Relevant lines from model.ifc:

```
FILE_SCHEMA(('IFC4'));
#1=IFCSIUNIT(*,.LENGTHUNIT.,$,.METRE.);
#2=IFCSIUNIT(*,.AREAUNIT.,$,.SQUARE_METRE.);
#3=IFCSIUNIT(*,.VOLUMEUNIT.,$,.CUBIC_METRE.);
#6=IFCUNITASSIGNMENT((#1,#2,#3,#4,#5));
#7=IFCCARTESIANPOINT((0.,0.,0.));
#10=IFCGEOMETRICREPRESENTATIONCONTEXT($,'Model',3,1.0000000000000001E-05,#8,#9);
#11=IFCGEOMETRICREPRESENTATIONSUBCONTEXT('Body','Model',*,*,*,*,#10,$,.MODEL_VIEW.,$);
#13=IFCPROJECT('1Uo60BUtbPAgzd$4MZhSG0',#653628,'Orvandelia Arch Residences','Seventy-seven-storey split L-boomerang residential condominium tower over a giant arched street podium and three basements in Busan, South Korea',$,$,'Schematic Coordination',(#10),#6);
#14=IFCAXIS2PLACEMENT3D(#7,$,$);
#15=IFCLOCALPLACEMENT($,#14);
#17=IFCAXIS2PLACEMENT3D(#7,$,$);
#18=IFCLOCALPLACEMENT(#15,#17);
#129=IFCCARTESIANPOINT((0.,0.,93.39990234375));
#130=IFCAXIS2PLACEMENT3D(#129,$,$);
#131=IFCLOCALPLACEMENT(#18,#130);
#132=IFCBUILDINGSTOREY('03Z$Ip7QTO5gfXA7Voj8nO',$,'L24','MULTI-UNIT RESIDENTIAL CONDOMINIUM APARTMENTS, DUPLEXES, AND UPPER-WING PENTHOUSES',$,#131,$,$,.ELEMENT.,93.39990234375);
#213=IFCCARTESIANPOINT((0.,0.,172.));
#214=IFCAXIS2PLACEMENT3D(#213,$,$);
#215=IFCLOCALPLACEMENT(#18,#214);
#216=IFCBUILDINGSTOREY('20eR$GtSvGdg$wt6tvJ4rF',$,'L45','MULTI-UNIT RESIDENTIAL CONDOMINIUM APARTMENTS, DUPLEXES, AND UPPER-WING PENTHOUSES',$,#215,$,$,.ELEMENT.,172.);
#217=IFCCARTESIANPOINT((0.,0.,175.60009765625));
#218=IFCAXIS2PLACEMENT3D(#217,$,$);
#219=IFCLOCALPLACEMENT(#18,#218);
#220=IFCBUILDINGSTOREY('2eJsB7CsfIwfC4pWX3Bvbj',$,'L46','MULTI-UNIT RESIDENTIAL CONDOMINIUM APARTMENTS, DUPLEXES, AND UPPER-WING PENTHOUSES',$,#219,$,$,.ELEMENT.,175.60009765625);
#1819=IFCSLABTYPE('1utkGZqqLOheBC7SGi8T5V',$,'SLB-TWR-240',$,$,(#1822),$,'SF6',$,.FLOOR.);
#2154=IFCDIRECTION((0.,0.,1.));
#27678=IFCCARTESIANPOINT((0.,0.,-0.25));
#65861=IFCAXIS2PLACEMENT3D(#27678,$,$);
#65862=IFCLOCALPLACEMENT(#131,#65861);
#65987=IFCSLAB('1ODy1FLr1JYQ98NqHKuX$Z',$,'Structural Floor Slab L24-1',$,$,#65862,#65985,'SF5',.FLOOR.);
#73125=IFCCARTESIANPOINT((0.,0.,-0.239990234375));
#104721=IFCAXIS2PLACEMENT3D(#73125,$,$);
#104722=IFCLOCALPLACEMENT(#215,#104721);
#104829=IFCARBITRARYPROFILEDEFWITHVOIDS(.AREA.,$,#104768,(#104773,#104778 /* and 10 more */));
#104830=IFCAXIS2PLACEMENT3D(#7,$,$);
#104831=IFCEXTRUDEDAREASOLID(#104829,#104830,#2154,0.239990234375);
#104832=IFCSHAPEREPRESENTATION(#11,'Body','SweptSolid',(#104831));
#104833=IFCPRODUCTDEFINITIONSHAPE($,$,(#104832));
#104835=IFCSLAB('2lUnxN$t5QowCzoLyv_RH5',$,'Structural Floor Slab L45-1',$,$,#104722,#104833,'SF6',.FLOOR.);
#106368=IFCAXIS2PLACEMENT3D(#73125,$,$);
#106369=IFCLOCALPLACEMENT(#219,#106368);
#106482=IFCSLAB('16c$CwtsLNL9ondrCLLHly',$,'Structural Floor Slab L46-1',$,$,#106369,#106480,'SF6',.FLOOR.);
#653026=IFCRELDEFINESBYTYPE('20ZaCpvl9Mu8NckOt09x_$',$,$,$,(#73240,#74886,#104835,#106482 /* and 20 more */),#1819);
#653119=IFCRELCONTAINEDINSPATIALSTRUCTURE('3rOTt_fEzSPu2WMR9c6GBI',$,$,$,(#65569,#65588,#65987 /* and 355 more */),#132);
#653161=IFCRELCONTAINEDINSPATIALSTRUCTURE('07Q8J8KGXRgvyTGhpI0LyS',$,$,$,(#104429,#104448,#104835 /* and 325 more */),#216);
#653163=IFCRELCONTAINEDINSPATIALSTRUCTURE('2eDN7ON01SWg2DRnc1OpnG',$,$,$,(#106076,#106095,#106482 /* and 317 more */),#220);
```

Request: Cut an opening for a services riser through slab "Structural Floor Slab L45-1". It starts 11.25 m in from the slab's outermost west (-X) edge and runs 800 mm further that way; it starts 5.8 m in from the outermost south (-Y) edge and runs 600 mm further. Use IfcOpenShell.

```python
import numpy as np
import ifcopenshell
import ifcopenshell.api.feature
import ifcopenshell.api.geometry
import ifcopenshell.api.root
import ifcopenshell.geom
import ifcopenshell.util.placement
import ifcopenshell.util.representation
import ifcopenshell.util.shape
import ifcopenshell.util.unit

model = ifcopenshell.open("model.ifc")
unit_scale = ifcopenshell.util.unit.calculate_unit_scale(model)
settings = ifcopenshell.geom.settings()


def volume(element):
    """Net volume in cubic metres, openings subtracted."""
    shape = ifcopenshell.geom.create_shape(settings, element)
    return ifcopenshell.util.shape.get_volume(shape.geometry)


slab = model.by_guid("2lUnxN$t5QowCzoLyv_RH5")
before = volume(slab)

# Extent in the slab's own axes, in metres. The edges named are its -X and -Y sides.
slab_shape = ifcopenshell.geom.create_shape(settings, slab)
vertices = ifcopenshell.util.shape.get_vertices(slab_shape.geometry)
x_min, y_min, bottom = vertices.min(axis=0)
top = vertices[:, 2].max()

opening = ifcopenshell.api.root.create_entity(model, ifc_class="IfcOpeningElement", name="Services riser opening", predefined_type="OPENING")
context = ifcopenshell.util.representation.get_context(model, "Model", "Body", "MODEL_VIEW")
width, depth = 0.8, 0.6
outline = [(0.0, 0.0), (width, 0.0), (width, depth), (0.0, depth), (0.0, 0.0)]
# Overshoot both faces by 50 mm so the cut is clean.
shape = ifcopenshell.api.geometry.add_slab_representation(
    model, context=context, depth=top - bottom + 0.1, polyline=outline
)
ifcopenshell.api.geometry.assign_representation(model, product=opening, representation=shape)

matrix = ifcopenshell.util.placement.get_local_placement(slab.ObjectPlacement)
matrix[:, 3] = matrix @ np.append(np.array([x_min + 11.25, y_min + 5.8, bottom - 0.05]) / unit_scale, 1.0)
ifcopenshell.api.geometry.edit_object_placement(model, product=opening, matrix=matrix, is_si=False)
ifcopenshell.api.feature.add_feature(model, feature=opening, element=slab)

after = volume(slab)

print(f"slab volume {before:.3f} -> {after:.3f} m3")

model.write("model_v2.ifc")
```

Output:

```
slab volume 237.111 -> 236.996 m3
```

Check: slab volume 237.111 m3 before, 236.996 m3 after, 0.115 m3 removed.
